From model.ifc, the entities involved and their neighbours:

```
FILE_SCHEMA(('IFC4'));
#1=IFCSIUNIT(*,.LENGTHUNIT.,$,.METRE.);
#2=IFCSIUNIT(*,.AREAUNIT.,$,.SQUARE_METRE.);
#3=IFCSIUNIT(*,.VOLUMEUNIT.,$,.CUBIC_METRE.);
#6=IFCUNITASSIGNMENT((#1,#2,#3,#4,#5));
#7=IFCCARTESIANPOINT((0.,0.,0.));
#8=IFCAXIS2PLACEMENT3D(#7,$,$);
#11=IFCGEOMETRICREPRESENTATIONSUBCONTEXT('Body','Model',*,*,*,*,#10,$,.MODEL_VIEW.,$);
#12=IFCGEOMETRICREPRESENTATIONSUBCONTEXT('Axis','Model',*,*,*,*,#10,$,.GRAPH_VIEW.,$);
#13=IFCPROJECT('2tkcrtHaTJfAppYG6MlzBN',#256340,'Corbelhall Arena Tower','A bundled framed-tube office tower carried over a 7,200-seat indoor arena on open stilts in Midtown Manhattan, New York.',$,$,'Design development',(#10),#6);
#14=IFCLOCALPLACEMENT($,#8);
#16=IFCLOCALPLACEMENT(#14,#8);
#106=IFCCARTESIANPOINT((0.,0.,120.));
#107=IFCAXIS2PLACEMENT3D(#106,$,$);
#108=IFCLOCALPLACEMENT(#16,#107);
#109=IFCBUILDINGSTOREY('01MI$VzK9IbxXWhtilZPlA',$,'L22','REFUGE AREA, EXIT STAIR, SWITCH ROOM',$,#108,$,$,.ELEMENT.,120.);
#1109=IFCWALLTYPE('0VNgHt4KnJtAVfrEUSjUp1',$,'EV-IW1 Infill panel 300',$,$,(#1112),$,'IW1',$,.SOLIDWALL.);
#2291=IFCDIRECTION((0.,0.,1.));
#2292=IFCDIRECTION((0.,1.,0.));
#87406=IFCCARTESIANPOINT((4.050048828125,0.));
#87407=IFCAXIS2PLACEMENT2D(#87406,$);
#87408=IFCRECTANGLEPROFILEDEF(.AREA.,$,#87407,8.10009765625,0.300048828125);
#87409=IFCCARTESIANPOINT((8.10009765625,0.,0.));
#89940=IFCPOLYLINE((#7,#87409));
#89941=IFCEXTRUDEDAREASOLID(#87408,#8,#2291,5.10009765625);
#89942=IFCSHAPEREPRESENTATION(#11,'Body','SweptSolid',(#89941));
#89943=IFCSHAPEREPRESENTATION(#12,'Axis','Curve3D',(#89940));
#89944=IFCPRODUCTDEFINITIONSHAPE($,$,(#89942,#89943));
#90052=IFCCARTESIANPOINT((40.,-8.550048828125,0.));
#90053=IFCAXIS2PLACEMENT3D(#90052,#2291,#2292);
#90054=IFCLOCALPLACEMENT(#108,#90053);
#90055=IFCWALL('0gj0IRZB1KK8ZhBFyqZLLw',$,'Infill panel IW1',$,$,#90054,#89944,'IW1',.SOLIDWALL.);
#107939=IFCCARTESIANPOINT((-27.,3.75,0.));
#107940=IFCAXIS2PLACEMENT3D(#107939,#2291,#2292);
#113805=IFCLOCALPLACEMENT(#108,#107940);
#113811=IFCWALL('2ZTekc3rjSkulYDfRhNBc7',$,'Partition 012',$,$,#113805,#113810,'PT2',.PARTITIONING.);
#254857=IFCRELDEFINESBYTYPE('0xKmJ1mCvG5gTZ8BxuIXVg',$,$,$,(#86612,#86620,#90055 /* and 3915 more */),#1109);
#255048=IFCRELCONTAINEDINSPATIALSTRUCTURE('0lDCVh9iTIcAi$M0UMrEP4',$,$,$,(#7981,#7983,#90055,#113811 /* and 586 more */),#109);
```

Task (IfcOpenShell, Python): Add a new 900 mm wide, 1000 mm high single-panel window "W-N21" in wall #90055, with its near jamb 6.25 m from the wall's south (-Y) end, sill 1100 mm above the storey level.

```python
import numpy as np
import ifcopenshell
import ifcopenshell.api.feature
import ifcopenshell.api.geometry
import ifcopenshell.api.root
import ifcopenshell.api.spatial
import ifcopenshell.geom
import ifcopenshell.util.element
import ifcopenshell.util.placement
import ifcopenshell.util.representation
import ifcopenshell.util.shape
import ifcopenshell.util.unit

model = ifcopenshell.open("model.ifc")
unit_scale = ifcopenshell.util.unit.calculate_unit_scale(model)
settings = ifcopenshell.geom.settings()


def volume(element):
    """Net volume in cubic metres, openings subtracted."""
    shape = ifcopenshell.geom.create_shape(settings, element)
    return ifcopenshell.util.shape.get_volume(shape.geometry)


wall = model.by_guid("0gj0IRZB1KK8ZhBFyqZLLw")
storey = ifcopenshell.util.element.get_container(wall, ifc_class="IfcBuildingStorey")
context = ifcopenshell.util.representation.get_context(model, "Model", "Body", "MODEL_VIEW")
before = volume(wall)

width, height, from_end, sill = 0.9, 1, 6.25, 1.1  # metres

# The wall runs along its own X axis, and the end named is its -X end.
wall_shape = ifcopenshell.geom.create_shape(settings, wall)
x, y, z = ifcopenshell.util.shape.get_vertices(wall_shape.geometry).T
start = x.min() + from_end
face, thickness = float(y.min()), float(y.max() - y.min())
wall_matrix = ifcopenshell.util.placement.get_local_placement(wall.ObjectPlacement)
level = ifcopenshell.util.placement.get_local_placement(storey.ObjectPlacement)[2, 3]


def in_wall(x, y):
    """Placement at x, y metres in the wall's axes, at sill height."""
    matrix = wall_matrix.copy()
    matrix[:, 3] = wall_matrix @ np.array([x / unit_scale, y / unit_scale, 0.0, 1.0])
    matrix[2, 3] = level + sill / unit_scale
    return matrix


# Opening: a box that overshoots both wall faces by 50 mm.
opening = ifcopenshell.api.root.create_entity(model, ifc_class="IfcOpeningElement", predefined_type="OPENING")
box = ifcopenshell.api.geometry.add_wall_representation(
    model, context=context, length=width, height=height, thickness=thickness + 0.1
)
ifcopenshell.api.geometry.assign_representation(model, product=opening, representation=box)
ifcopenshell.api.geometry.edit_object_placement(model, product=opening, matrix=in_wall(start, face - 0.05), is_si=False)
ifcopenshell.api.feature.add_feature(model, feature=opening, element=wall)

window = ifcopenshell.api.root.create_entity(model, ifc_class="IfcWindow", name="W-N21", predefined_type="WINDOW")
window.OverallWidth, window.OverallHeight = width / unit_scale, height / unit_scale
window.PartitioningType = "SINGLE_PANEL"
body = ifcopenshell.api.geometry.add_window_representation(
    model,
    context=context,
    overall_width=window.OverallWidth,
    overall_height=window.OverallHeight,
    partition_type="SINGLE_PANEL",
)
ifcopenshell.api.geometry.assign_representation(model, product=window, representation=body)
ifcopenshell.api.spatial.assign_container(model, products=[window], relating_structure=storey)
ifcopenshell.api.feature.add_filling(model, opening=opening, element=window)

# Centre the window in the wall's thickness.
ifcopenshell.api.geometry.edit_object_placement(model, product=window, matrix=in_wall(start, face), is_si=False)
window_shape = ifcopenshell.geom.create_shape(settings, window)
depth = ifcopenshell.util.shape.get_vertices(window_shape.geometry)[:, 1]
offset = face + thickness / 2 - (depth.min() + depth.max()) / 2
ifcopenshell.api.geometry.edit_object_placement(model, product=window, matrix=in_wall(start, offset), is_si=False)

after = volume(wall)

print(f"wall volume {before:.3f} -> {after:.3f} m3")

model.write("model_updated.ifc")
```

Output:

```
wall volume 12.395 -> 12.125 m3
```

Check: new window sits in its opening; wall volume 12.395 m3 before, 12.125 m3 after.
